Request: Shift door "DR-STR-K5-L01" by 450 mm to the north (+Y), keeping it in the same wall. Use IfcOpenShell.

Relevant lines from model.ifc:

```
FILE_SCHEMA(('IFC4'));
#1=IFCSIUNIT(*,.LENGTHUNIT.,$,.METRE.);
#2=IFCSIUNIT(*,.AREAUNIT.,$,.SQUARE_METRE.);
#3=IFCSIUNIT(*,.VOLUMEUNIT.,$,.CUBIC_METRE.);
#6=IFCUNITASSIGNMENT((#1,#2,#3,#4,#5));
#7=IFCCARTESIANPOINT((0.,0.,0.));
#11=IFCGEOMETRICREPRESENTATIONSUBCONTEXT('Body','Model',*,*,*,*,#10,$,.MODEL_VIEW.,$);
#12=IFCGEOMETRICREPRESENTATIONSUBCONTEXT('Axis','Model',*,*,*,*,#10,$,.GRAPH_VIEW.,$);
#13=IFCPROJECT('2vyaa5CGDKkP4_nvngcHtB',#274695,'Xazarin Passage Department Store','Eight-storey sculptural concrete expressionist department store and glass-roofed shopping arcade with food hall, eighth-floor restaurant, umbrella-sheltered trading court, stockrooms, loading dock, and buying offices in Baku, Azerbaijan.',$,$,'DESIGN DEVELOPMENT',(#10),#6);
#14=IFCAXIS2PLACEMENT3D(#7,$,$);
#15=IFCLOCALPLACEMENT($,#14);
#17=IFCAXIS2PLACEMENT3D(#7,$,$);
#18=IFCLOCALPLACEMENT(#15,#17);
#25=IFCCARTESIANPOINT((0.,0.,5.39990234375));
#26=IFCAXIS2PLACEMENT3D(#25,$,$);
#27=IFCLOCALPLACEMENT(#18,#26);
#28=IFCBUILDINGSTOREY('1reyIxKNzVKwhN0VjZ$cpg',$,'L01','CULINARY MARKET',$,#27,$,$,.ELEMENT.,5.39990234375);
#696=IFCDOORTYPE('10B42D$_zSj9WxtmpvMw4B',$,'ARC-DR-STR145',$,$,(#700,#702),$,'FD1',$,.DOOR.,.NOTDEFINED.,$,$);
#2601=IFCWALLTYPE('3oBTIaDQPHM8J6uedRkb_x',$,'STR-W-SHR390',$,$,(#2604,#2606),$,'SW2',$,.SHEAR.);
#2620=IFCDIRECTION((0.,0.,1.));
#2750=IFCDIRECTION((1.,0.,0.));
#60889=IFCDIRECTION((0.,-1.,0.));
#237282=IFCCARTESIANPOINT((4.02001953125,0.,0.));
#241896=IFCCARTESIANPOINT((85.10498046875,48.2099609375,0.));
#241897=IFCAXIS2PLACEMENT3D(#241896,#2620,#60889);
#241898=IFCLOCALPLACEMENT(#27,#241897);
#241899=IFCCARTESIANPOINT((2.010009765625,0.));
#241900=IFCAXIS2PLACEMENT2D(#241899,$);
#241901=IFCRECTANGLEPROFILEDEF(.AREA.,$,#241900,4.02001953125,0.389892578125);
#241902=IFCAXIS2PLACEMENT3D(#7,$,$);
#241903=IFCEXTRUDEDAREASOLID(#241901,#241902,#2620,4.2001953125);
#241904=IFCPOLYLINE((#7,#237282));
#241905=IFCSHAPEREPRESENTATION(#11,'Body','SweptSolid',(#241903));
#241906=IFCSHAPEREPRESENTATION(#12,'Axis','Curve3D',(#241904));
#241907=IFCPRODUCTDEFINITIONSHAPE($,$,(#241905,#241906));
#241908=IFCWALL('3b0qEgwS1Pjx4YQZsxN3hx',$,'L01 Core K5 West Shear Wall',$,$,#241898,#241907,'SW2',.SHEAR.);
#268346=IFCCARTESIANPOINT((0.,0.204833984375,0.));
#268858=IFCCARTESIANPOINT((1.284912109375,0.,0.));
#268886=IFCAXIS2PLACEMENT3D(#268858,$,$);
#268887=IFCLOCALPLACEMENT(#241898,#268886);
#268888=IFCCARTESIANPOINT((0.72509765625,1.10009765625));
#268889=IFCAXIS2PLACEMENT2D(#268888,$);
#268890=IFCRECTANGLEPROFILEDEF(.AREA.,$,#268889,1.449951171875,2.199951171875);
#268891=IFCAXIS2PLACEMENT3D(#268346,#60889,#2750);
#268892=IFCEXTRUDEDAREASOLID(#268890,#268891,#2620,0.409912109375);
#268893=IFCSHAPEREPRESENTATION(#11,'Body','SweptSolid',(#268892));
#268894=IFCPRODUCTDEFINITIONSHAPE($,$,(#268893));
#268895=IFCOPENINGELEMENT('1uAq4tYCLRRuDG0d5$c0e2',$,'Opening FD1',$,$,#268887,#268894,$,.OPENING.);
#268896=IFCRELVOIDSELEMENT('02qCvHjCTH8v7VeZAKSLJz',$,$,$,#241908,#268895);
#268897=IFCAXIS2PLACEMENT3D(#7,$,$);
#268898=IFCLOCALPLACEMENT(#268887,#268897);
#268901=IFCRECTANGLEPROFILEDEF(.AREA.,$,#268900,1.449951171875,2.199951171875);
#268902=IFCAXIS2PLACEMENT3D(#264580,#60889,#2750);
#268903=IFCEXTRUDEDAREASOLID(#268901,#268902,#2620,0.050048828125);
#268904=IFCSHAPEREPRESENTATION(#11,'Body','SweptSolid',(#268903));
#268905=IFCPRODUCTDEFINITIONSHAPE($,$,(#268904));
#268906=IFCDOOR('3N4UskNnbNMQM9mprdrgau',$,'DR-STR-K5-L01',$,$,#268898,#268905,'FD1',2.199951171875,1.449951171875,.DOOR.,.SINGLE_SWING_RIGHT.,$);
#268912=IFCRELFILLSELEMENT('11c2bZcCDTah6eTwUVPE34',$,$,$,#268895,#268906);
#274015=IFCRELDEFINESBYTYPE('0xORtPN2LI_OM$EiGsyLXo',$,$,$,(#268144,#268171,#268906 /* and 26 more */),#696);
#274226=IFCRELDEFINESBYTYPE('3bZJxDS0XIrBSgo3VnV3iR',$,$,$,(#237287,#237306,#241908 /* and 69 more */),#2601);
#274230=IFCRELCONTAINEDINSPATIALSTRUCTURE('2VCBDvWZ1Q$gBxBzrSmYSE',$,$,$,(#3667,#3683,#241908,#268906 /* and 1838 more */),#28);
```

```python
import ifcopenshell
import ifcopenshell.api.geometry
import ifcopenshell.util.placement
import ifcopenshell.util.unit

model = ifcopenshell.open("model.ifc")
unit_scale = ifcopenshell.util.unit.calculate_unit_scale(model)

door = model.by_guid("3N4UskNnbNMQM9mprdrgau")
opening = door.FillsVoids[0].RelatingOpeningElement
wall = opening.VoidsElements[0].RelatingBuildingElement

wall_matrix = ifcopenshell.util.placement.get_local_placement(wall.ObjectPlacement)
shift = wall_matrix[:3, 0] * -0.45 / unit_scale
before = ifcopenshell.util.placement.get_local_placement(door.ObjectPlacement)[:3, 3].copy()

# The door is placed relative to its opening, so it follows when the opening moves.
matrix = ifcopenshell.util.placement.get_local_placement(opening.ObjectPlacement)
matrix[:3, 3] += shift
ifcopenshell.api.geometry.edit_object_placement(
    model, product=opening, matrix=matrix, is_si=False, should_transform_children=True
)

after = ifcopenshell.util.placement.get_local_placement(door.ObjectPlacement)[:3, 3]
print("door moved by", (after - before).round(3) + 0.0)

model.write("model_updated.ifc")
```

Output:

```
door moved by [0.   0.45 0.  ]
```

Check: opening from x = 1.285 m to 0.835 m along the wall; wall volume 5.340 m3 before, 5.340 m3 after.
